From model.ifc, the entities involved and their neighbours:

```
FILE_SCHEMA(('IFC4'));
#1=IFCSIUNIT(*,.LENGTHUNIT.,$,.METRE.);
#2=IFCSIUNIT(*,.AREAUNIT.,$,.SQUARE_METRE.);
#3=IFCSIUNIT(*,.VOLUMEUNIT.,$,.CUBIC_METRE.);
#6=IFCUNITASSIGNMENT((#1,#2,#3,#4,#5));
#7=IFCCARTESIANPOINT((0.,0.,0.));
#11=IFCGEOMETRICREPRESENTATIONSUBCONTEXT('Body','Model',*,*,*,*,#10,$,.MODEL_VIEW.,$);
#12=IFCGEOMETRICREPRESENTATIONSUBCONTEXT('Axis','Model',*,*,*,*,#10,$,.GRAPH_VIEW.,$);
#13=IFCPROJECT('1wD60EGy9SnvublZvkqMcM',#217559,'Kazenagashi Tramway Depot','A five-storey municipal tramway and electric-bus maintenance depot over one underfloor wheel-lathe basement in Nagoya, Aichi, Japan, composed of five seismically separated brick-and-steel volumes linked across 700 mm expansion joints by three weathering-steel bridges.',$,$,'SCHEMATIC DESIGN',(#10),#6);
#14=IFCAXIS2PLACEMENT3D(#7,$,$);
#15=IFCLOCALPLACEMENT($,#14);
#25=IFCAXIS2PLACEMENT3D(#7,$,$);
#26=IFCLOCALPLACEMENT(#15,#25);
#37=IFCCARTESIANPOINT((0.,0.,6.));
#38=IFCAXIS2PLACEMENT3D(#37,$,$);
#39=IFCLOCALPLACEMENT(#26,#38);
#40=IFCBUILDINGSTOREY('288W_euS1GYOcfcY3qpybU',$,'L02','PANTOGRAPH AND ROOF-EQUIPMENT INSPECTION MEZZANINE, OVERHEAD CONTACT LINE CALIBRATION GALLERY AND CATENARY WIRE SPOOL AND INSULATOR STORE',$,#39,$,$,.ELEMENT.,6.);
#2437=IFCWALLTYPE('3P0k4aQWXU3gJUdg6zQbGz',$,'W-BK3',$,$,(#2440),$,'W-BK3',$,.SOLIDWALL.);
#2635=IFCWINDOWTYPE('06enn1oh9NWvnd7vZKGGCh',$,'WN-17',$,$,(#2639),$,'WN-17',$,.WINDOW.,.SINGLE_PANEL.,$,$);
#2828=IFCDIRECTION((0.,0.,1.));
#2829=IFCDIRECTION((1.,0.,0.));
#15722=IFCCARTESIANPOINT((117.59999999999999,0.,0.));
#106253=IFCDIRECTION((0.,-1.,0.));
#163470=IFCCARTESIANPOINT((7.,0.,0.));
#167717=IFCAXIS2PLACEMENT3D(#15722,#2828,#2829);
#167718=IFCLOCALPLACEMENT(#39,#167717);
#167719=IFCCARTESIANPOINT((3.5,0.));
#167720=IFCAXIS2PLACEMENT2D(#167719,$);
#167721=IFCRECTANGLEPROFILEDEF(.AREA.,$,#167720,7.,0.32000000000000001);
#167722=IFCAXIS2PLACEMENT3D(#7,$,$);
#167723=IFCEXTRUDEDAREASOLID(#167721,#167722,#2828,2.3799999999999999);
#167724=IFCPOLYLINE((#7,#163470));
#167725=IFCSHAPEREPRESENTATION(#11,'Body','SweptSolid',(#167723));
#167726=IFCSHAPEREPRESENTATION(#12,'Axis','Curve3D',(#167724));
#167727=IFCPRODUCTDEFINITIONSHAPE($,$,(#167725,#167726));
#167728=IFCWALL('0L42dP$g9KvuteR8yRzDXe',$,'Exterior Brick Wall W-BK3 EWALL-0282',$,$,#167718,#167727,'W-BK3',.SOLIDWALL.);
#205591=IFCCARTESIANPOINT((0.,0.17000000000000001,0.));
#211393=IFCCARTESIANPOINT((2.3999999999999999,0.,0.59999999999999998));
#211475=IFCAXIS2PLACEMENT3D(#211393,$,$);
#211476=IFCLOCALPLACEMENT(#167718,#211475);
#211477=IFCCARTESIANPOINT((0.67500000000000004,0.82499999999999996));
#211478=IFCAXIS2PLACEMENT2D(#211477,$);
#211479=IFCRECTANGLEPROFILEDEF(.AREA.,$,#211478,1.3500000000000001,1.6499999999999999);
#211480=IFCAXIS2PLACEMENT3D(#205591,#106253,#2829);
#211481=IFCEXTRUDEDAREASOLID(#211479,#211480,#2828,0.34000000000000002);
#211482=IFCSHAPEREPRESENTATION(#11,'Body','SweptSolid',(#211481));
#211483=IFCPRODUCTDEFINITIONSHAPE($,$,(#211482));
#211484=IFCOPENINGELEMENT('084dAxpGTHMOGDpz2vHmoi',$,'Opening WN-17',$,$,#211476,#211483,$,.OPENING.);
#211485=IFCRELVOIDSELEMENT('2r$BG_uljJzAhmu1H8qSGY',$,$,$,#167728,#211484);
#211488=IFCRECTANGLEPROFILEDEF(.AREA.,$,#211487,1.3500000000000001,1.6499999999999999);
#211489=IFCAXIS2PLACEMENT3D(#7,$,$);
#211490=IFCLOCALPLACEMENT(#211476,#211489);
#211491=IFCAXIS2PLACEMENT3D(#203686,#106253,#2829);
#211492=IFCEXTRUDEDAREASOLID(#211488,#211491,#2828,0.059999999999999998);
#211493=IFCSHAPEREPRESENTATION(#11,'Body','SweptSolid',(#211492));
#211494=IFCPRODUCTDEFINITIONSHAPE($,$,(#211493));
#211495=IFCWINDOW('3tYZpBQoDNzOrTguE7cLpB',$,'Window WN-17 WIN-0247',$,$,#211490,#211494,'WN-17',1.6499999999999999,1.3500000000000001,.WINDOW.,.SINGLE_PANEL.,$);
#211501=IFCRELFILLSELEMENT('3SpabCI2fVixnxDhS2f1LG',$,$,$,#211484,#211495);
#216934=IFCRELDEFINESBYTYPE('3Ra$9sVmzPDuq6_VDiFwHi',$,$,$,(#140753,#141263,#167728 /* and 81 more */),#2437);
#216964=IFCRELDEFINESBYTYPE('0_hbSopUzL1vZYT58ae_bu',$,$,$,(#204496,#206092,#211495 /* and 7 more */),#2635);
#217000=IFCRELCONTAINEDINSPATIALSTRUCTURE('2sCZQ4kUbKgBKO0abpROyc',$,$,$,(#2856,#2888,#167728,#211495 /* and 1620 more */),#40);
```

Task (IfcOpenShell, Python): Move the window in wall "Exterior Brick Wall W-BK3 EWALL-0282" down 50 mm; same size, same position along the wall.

```python
import numpy as np
import ifcopenshell
import ifcopenshell.api.geometry
import ifcopenshell.util.placement
import ifcopenshell.util.unit

model = ifcopenshell.open("model.ifc")
unit_scale = ifcopenshell.util.unit.calculate_unit_scale(model)

window = model.by_id(211495)
opening = window.FillsVoids[0].RelatingOpeningElement
dz = -0.05 / unit_scale

shift = np.array([0.0, 0.0, dz])
# The window is placed relative to its opening, so it follows when the opening moves.
matrix = ifcopenshell.util.placement.get_local_placement(opening.ObjectPlacement)
matrix[:3, 3] += shift
ifcopenshell.api.geometry.edit_object_placement(
    model, product=opening, matrix=matrix, is_si=False, should_transform_children=True
)

print(f"moved by {dz * unit_scale:+.3f} m")

model.write("model_updated.ifc")
```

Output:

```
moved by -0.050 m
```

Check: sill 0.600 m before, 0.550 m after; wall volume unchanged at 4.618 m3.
